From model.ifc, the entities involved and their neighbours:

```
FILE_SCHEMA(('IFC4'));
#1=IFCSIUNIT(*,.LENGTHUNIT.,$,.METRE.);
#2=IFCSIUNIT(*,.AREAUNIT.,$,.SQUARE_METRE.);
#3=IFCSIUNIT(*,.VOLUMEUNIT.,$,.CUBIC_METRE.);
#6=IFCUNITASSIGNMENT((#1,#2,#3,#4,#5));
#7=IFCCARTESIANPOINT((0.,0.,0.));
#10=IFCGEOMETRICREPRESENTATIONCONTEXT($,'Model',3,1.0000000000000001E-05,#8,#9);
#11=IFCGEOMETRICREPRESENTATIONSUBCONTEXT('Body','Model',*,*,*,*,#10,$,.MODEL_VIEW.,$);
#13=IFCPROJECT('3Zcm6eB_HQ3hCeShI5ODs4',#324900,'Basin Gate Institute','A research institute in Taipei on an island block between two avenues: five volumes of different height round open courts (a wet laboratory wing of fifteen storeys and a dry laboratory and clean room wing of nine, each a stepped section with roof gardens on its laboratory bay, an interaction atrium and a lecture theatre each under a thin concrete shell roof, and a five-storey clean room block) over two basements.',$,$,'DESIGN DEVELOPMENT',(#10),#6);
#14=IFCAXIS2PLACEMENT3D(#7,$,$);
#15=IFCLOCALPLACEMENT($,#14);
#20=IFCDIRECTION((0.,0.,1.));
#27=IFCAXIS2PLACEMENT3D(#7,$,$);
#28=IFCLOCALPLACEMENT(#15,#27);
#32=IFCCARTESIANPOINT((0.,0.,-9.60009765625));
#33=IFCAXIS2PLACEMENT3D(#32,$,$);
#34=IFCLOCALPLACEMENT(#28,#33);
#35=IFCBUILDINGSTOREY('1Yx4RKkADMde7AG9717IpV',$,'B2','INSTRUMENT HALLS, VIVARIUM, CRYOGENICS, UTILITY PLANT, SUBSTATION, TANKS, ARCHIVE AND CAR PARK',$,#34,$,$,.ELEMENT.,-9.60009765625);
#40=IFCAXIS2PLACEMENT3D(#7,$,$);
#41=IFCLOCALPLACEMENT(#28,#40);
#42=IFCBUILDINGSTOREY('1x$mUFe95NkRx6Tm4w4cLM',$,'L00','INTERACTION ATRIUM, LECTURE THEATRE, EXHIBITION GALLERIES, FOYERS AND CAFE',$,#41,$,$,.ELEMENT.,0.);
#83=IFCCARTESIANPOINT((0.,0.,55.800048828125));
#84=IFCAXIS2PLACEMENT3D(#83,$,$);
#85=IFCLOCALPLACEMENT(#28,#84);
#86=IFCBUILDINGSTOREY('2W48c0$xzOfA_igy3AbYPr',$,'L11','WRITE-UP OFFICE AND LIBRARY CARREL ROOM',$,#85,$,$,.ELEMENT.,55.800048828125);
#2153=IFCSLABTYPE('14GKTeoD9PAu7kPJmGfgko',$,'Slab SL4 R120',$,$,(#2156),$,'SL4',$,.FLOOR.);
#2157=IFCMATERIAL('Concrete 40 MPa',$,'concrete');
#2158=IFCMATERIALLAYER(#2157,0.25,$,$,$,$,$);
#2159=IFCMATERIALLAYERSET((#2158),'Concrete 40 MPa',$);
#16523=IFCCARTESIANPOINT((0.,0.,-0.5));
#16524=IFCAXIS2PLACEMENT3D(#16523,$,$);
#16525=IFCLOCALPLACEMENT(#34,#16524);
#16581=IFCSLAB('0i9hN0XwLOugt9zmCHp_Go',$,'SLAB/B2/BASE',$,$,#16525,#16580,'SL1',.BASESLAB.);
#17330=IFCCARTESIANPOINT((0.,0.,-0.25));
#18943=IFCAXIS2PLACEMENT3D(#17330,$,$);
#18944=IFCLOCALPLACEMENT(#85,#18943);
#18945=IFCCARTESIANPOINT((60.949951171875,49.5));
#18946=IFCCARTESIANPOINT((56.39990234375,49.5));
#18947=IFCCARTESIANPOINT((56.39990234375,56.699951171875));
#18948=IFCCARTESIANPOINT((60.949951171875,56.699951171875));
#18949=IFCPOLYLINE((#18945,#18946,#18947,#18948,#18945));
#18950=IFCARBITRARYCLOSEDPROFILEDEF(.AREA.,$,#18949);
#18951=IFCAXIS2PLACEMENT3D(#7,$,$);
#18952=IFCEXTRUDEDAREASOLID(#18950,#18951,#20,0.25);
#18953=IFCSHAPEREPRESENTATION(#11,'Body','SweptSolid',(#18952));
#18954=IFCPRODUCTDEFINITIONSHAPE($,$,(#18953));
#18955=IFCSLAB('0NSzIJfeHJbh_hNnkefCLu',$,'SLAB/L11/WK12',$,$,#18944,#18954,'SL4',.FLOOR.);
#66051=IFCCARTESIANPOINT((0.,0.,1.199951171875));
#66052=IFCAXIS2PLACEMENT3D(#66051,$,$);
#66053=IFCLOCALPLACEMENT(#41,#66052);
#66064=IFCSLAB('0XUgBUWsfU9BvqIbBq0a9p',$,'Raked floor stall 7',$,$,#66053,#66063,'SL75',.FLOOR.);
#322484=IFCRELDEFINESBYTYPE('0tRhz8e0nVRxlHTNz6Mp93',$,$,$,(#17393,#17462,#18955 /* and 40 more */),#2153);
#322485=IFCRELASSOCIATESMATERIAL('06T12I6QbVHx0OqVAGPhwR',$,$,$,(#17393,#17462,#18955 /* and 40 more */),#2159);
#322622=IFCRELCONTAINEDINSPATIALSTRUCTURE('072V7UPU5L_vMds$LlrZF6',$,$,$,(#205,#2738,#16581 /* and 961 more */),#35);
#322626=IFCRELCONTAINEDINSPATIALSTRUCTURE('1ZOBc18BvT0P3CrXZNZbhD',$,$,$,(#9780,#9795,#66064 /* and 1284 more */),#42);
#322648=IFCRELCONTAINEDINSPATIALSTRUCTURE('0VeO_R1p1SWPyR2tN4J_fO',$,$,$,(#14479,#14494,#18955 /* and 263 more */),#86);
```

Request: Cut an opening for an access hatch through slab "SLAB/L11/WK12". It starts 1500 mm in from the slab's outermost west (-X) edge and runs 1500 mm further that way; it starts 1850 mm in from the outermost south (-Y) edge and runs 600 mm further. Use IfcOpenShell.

```python
import numpy as np
import ifcopenshell
import ifcopenshell.api.feature
import ifcopenshell.api.geometry
import ifcopenshell.api.root
import ifcopenshell.geom
import ifcopenshell.util.placement
import ifcopenshell.util.representation
import ifcopenshell.util.shape
import ifcopenshell.util.unit

model = ifcopenshell.open("model.ifc")
unit_scale = ifcopenshell.util.unit.calculate_unit_scale(model)
settings = ifcopenshell.geom.settings()


def volume(element):
    """Net volume in cubic metres, openings subtracted."""
    shape = ifcopenshell.geom.create_shape(settings, element)
    return ifcopenshell.util.shape.get_volume(shape.geometry)


slab = model.by_guid("0NSzIJfeHJbh_hNnkefCLu")
before = volume(slab)

# Extent in the slab's own axes, in metres. The edges named are its -X and -Y sides.
slab_shape = ifcopenshell.geom.create_shape(settings, slab)
vertices = ifcopenshell.util.shape.get_vertices(slab_shape.geometry)
x_min, y_min, bottom = vertices.min(axis=0)
top = vertices[:, 2].max()

opening = ifcopenshell.api.root.create_entity(model, ifc_class="IfcOpeningElement", name="Access hatch opening", predefined_type="OPENING")
context = ifcopenshell.util.representation.get_context(model, "Model", "Body", "MODEL_VIEW")
width, depth = 1.5, 0.6
outline = [(0.0, 0.0), (width, 0.0), (width, depth), (0.0, depth), (0.0, 0.0)]
# Overshoot both faces by 50 mm so the cut is clean.
shape = ifcopenshell.api.geometry.add_slab_representation(
    model, context=context, depth=top - bottom + 0.1, polyline=outline
)
ifcopenshell.api.geometry.assign_representation(model, product=opening, representation=shape)

matrix = ifcopenshell.util.placement.get_local_placement(slab.ObjectPlacement)
matrix[:, 3] = matrix @ np.append(np.array([x_min + 1.5, y_min + 1.85, bottom - 0.05]) / unit_scale, 1.0)
ifcopenshell.api.geometry.edit_object_placement(model, product=opening, matrix=matrix, is_si=False)
ifcopenshell.api.feature.add_feature(model, feature=opening, element=slab)

after = volume(slab)

print(f"slab volume {before:.3f} -> {after:.3f} m3")

model.write("model_edited.ifc")
```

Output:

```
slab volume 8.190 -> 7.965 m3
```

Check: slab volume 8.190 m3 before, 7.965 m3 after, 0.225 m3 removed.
